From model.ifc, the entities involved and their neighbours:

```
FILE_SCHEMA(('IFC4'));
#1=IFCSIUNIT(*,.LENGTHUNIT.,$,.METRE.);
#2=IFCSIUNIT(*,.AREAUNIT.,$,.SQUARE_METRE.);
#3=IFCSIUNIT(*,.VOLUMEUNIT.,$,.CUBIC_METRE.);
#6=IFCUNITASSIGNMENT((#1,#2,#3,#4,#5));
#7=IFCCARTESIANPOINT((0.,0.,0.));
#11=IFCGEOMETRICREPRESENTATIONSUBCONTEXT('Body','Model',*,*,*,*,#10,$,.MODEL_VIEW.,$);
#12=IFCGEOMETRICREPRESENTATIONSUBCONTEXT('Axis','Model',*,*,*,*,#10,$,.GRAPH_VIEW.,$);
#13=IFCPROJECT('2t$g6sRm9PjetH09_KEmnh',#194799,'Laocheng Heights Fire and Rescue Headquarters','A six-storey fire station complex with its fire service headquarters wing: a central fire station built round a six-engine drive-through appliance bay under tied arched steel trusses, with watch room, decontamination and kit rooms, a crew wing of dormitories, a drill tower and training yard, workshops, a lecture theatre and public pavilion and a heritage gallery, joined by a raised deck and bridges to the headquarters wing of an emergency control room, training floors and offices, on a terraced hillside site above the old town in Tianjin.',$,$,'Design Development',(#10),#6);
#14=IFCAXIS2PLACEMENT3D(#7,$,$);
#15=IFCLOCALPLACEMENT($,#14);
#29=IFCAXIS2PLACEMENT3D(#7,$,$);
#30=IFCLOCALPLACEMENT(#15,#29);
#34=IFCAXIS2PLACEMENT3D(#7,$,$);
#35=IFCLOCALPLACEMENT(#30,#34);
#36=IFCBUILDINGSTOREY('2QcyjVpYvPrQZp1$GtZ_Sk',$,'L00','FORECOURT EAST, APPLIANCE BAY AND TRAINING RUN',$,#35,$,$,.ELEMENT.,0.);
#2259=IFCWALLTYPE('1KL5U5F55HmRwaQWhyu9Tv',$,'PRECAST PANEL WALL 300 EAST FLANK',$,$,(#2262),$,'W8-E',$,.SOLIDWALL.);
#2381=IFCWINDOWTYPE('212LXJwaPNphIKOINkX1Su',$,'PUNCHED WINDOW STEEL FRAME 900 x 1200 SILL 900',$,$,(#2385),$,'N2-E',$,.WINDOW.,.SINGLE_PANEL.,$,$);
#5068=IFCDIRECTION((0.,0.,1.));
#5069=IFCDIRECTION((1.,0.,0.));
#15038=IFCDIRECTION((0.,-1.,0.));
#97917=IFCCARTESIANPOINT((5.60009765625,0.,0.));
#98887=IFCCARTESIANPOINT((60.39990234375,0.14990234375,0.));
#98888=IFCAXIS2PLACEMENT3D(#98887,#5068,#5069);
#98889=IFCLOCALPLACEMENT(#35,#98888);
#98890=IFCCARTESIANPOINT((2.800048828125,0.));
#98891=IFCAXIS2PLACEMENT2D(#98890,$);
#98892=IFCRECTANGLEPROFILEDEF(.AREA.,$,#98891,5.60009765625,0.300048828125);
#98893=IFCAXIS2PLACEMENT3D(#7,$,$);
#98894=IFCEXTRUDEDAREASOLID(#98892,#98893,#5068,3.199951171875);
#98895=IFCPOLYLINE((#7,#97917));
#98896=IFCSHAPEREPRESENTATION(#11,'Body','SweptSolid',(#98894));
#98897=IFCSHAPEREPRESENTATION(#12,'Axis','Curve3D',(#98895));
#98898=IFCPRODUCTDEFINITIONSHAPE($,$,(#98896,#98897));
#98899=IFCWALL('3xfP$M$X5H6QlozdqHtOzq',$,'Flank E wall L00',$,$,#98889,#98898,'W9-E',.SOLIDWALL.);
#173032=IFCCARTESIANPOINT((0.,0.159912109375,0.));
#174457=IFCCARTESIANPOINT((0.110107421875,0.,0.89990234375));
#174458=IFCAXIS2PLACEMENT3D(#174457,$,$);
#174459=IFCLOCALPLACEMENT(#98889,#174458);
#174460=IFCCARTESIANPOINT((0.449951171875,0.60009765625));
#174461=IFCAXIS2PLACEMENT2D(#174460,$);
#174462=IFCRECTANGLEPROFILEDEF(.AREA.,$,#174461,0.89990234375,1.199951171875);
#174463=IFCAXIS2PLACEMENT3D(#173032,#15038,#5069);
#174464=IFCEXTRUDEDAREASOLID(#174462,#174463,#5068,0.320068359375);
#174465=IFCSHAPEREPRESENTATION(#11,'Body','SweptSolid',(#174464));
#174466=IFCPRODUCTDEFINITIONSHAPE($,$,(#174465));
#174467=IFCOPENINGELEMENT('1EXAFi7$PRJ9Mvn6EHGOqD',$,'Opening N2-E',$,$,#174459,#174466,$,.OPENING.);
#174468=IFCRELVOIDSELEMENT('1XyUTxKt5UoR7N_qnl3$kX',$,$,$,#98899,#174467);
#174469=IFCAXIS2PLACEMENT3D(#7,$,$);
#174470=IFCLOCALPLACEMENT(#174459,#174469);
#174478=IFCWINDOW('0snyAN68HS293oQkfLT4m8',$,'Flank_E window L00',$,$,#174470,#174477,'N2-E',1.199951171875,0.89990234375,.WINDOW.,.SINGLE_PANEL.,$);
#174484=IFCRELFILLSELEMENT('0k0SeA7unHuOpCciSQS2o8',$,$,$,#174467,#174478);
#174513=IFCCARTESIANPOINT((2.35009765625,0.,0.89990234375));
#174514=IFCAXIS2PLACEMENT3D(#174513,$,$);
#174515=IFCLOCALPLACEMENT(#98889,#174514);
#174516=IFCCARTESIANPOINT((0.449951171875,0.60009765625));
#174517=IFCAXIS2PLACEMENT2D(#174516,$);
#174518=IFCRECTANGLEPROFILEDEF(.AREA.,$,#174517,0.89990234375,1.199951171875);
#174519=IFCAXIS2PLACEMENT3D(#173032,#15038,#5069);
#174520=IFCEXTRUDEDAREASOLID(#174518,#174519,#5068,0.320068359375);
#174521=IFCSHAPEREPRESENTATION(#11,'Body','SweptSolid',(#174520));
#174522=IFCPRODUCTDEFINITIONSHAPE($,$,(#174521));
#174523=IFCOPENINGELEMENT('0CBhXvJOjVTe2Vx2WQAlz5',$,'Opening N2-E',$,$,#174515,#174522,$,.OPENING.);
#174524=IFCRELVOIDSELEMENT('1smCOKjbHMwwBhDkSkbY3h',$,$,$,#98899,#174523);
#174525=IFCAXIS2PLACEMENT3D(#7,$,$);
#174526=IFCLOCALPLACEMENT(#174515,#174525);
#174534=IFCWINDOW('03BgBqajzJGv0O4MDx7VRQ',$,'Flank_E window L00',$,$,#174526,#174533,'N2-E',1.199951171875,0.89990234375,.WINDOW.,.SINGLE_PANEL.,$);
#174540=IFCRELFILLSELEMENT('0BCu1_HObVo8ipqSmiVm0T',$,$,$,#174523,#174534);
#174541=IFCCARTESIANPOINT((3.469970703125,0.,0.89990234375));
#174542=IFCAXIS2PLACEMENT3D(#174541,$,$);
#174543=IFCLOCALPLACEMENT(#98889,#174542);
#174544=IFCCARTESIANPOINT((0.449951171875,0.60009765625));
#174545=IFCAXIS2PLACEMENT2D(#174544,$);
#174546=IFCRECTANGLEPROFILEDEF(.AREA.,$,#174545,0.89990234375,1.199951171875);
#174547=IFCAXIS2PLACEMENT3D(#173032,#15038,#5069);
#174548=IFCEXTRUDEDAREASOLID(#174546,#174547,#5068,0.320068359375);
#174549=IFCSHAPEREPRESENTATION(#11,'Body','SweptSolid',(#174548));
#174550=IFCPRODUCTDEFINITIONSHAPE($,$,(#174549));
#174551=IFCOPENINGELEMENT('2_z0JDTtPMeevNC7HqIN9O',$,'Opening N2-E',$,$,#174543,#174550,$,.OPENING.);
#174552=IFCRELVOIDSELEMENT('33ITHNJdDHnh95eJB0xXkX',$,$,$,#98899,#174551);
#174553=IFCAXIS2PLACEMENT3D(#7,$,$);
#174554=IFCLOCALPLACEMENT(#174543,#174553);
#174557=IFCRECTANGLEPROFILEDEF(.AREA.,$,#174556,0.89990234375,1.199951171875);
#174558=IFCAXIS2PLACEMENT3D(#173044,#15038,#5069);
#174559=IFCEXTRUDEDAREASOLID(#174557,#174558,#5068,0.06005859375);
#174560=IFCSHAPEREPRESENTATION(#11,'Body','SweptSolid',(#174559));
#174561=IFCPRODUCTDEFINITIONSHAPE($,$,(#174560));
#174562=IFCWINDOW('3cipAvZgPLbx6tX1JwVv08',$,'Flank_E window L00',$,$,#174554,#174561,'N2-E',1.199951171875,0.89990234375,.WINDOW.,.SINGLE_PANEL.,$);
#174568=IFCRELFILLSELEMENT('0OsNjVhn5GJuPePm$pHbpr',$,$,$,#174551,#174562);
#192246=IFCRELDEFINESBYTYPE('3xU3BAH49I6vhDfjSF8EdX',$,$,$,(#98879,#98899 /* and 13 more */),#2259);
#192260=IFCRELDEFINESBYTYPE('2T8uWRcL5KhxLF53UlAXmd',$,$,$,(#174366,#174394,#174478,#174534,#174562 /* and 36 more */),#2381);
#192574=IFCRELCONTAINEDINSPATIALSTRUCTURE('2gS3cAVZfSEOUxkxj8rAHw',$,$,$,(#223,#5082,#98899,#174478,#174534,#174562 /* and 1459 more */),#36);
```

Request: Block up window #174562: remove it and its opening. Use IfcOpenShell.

```python
import ifcopenshell
import ifcopenshell.api.feature
import ifcopenshell.api.root
import ifcopenshell.geom
import ifcopenshell.util.shape

model = ifcopenshell.open("model.ifc")
settings = ifcopenshell.geom.settings()


def volume(element):
    """Net volume in cubic metres, openings subtracted."""
    shape = ifcopenshell.geom.create_shape(settings, element)
    return ifcopenshell.util.shape.get_volume(shape.geometry)


window = model.by_guid("3cipAvZgPLbx6tX1JwVv08")
opening = window.FillsVoids[0].RelatingOpeningElement
wall = opening.VoidsElements[0].RelatingBuildingElement
before = volume(wall)

ifcopenshell.api.root.remove_product(model, product=window)
ifcopenshell.api.feature.remove_feature(model, feature=opening)

after = volume(wall)

print(f"wall volume {before:.3f} -> {after:.3f} m3")

model.write("model_v2.ifc")
```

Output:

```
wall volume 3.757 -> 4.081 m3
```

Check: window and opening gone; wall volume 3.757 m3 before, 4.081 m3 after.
